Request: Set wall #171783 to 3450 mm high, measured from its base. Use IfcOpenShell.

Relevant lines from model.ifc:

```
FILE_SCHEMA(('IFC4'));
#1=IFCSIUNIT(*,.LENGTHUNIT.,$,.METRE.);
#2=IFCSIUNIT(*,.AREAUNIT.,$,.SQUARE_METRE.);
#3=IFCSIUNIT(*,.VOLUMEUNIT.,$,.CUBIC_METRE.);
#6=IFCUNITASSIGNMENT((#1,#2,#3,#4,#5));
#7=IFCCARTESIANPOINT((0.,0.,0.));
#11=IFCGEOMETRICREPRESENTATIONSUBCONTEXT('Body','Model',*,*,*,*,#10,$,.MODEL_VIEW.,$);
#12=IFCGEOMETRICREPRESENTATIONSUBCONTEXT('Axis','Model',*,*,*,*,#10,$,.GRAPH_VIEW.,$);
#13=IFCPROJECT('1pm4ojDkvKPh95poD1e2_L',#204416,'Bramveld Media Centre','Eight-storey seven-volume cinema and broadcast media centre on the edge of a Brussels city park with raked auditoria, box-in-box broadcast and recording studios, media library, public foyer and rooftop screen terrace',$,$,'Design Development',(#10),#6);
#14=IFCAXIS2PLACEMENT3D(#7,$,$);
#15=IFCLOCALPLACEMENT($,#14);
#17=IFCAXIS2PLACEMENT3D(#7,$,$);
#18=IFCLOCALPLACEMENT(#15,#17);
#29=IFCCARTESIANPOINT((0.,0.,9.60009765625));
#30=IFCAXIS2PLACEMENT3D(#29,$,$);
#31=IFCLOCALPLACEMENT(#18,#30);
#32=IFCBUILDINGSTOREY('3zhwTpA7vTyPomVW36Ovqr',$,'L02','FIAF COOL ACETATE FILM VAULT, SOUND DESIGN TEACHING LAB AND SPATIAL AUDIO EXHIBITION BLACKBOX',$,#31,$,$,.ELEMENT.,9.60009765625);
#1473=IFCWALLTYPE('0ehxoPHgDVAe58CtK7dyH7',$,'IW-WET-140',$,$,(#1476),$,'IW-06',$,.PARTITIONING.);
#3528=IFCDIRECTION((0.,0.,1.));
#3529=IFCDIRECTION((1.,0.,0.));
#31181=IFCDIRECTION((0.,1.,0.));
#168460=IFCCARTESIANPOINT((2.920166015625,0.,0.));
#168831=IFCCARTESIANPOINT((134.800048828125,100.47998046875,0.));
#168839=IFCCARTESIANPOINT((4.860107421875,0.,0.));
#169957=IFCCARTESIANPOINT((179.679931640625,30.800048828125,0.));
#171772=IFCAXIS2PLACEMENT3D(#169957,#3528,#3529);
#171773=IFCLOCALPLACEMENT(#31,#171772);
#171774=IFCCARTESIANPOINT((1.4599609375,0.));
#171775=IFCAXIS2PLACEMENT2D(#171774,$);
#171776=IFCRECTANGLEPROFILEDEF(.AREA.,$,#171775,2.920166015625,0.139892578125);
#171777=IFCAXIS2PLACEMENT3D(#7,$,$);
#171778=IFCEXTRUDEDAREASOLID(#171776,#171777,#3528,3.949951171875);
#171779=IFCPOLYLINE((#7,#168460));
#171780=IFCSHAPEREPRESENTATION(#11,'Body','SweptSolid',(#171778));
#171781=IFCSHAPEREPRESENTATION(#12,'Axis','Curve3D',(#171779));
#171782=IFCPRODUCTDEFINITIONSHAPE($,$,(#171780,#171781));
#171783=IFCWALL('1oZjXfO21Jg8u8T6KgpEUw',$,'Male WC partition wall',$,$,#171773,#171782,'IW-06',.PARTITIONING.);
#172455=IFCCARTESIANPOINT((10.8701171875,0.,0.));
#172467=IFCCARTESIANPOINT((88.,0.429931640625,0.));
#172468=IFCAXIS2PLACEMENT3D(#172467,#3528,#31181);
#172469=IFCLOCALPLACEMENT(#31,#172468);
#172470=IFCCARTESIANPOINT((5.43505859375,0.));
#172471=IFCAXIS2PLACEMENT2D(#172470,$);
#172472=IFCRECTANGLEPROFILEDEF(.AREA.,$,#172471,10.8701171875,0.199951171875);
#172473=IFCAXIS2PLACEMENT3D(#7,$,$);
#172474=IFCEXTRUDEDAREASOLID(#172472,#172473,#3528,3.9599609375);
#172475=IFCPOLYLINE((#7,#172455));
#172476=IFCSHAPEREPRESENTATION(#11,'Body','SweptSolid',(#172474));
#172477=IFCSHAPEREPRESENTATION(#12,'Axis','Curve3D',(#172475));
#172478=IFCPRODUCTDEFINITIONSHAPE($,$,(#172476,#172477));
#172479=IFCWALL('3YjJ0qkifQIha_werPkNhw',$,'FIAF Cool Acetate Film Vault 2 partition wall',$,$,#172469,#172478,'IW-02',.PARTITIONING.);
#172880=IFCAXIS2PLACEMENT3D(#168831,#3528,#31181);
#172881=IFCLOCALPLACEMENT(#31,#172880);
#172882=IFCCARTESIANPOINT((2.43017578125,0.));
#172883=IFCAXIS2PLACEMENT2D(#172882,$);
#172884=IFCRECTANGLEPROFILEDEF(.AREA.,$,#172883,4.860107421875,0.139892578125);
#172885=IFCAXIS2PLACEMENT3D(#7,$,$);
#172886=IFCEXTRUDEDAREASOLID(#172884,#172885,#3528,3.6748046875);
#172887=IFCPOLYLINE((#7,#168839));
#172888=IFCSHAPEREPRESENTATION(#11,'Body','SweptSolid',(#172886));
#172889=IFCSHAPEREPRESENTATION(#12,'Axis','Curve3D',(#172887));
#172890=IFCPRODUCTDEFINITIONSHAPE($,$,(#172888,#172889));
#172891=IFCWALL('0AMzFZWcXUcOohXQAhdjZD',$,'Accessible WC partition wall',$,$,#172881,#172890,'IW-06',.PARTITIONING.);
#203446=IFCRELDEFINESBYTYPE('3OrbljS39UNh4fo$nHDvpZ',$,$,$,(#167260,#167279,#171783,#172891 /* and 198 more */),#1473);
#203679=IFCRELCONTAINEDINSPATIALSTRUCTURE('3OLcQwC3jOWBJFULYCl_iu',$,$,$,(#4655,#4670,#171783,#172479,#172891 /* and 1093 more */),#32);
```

```python
import ifcopenshell
import ifcopenshell.geom
import ifcopenshell.util.representation
import ifcopenshell.util.shape
import ifcopenshell.util.unit

model = ifcopenshell.open("model.ifc")
unit_scale = ifcopenshell.util.unit.calculate_unit_scale(model)
settings = ifcopenshell.geom.settings()


def volume(element):
    """Net volume in cubic metres, openings subtracted."""
    shape = ifcopenshell.geom.create_shape(settings, element)
    return ifcopenshell.util.shape.get_volume(shape.geometry)


wall = model.by_id(171783)
before = volume(wall)

body = ifcopenshell.util.representation.get_representation(wall, "Model", "Body")
solid = body.Items[0]
old_height = solid.Depth
solid.Depth = 3.45 / unit_scale
after = volume(wall)

print(f"height {old_height:g} -> {solid.Depth:g}, volume {before:.3f} -> {after:.3f} m3")

model.write("model_updated.ifc")
```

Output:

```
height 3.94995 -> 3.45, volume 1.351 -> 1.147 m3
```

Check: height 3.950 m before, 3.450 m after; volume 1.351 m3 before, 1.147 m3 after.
